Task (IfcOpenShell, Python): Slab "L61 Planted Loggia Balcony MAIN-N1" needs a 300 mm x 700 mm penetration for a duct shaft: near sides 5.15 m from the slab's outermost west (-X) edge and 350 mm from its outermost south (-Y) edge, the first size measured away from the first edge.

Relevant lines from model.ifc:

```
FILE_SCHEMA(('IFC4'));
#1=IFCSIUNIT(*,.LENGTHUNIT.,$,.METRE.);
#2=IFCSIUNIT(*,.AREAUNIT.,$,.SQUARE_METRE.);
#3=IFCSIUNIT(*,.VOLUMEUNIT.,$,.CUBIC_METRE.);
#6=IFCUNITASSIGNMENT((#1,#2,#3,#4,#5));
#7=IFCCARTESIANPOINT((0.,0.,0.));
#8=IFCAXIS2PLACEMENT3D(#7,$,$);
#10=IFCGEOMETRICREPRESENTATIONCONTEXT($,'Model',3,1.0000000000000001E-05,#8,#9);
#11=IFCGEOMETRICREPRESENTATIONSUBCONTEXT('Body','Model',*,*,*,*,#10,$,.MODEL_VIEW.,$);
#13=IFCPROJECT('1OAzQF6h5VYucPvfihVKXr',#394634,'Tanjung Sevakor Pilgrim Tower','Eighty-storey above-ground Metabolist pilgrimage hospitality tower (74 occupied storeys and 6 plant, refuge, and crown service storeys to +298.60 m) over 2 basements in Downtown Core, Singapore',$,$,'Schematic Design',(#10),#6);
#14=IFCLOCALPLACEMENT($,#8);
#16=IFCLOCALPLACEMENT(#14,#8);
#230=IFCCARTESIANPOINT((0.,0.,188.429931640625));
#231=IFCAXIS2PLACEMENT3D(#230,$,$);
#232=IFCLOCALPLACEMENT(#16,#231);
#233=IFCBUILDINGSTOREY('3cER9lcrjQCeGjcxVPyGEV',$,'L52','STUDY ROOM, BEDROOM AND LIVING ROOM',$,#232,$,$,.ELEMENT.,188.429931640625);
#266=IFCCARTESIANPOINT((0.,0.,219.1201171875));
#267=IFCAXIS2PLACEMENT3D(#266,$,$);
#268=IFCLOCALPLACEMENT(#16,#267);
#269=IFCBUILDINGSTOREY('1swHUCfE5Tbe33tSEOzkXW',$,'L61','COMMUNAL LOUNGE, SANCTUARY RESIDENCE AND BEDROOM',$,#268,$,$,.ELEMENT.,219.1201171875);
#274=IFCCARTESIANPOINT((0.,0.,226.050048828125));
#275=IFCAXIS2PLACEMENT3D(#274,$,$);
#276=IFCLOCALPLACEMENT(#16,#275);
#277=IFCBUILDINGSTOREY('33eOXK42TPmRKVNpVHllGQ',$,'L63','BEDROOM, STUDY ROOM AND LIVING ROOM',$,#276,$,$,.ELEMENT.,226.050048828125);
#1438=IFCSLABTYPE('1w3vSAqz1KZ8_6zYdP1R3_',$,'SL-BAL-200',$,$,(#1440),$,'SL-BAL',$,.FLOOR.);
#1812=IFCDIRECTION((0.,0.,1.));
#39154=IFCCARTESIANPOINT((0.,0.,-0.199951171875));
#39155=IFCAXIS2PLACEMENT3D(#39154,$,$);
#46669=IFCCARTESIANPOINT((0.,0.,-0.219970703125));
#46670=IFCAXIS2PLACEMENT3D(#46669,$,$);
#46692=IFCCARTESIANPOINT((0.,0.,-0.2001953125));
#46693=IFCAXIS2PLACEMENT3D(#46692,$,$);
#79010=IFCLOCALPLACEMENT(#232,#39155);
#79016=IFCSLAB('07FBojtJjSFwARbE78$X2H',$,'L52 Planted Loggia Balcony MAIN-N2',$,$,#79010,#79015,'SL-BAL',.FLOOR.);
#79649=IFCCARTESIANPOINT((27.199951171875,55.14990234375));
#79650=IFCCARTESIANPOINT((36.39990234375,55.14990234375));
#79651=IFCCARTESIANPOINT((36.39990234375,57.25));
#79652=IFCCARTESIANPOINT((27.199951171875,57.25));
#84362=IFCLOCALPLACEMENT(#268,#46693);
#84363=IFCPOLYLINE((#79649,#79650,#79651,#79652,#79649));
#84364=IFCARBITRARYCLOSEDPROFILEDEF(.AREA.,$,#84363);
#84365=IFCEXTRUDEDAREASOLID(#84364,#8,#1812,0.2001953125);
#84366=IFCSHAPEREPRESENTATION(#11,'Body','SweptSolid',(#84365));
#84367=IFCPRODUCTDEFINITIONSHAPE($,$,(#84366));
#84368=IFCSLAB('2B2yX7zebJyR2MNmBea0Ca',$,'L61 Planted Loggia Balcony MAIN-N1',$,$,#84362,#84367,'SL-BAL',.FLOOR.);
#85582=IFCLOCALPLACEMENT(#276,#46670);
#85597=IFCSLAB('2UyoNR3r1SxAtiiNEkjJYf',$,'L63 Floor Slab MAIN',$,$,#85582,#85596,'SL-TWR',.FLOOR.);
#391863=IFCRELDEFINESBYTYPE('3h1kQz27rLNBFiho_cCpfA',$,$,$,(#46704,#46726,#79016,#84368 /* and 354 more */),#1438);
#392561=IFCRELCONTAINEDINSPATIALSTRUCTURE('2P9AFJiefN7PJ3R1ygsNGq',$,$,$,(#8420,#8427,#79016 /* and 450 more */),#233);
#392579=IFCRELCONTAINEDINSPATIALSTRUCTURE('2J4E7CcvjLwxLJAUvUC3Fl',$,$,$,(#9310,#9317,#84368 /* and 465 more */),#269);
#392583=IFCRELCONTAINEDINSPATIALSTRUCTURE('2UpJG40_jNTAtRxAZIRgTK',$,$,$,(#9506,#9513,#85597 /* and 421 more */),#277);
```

```python
import numpy as np
import ifcopenshell
import ifcopenshell.api.feature
import ifcopenshell.api.geometry
import ifcopenshell.api.root
import ifcopenshell.geom
import ifcopenshell.util.placement
import ifcopenshell.util.representation
import ifcopenshell.util.shape
import ifcopenshell.util.unit

model = ifcopenshell.open("model.ifc")
unit_scale = ifcopenshell.util.unit.calculate_unit_scale(model)
settings = ifcopenshell.geom.settings()


def volume(element):
    """Net volume in cubic metres, openings subtracted."""
    shape = ifcopenshell.geom.create_shape(settings, element)
    return ifcopenshell.util.shape.get_volume(shape.geometry)


slab = model.by_guid("2B2yX7zebJyR2MNmBea0Ca")
before = volume(slab)

# Extent in the slab's own axes, in metres. The edges named are its -X and -Y sides.
slab_shape = ifcopenshell.geom.create_shape(settings, slab)
vertices = ifcopenshell.util.shape.get_vertices(slab_shape.geometry)
x_min, y_min, bottom = vertices.min(axis=0)
top = vertices[:, 2].max()

opening = ifcopenshell.api.root.create_entity(model, ifc_class="IfcOpeningElement", name="Duct shaft opening", predefined_type="OPENING")
context = ifcopenshell.util.representation.get_context(model, "Model", "Body", "MODEL_VIEW")
width, depth = 0.3, 0.7
outline = [(0.0, 0.0), (width, 0.0), (width, depth), (0.0, depth), (0.0, 0.0)]
# Overshoot both faces by 50 mm so the cut is clean.
shape = ifcopenshell.api.geometry.add_slab_representation(
    model, context=context, depth=top - bottom + 0.1, polyline=outline
)
ifcopenshell.api.geometry.assign_representation(model, product=opening, representation=shape)

matrix = ifcopenshell.util.placement.get_local_placement(slab.ObjectPlacement)
matrix[:, 3] = matrix @ np.append(np.array([x_min + 5.15, y_min + 0.35, bottom - 0.05]) / unit_scale, 1.0)
ifcopenshell.api.geometry.edit_object_placement(model, product=opening, matrix=matrix, is_si=False)
ifcopenshell.api.feature.add_feature(model, feature=opening, element=slab)

after = volume(slab)

print(f"slab volume {before:.3f} -> {after:.3f} m3")

model.write("model-out.ifc")
```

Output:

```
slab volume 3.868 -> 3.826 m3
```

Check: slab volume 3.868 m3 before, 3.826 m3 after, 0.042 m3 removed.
